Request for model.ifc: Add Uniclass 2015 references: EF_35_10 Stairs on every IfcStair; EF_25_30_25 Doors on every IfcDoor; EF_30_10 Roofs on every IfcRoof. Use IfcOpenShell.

First a look at what the model holds.

```python
import ifcopenshell

model = ifcopenshell.open("model.ifc")
print(model.schema)
print("classifications:", [c.Name for c in model.by_type("IfcClassification")])
for ifc_class in ("IfcDoor", "IfcRoof", "IfcStair", "IfcWall", "IfcWindow"):
    print(ifc_class, len(model.by_type(ifc_class)))
```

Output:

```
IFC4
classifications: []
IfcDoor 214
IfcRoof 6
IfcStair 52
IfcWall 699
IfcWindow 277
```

```python
import ifcopenshell
import ifcopenshell.api.classification

model = ifcopenshell.open("model.ifc")

system = ifcopenshell.api.classification.add_classification(model, classification="Uniclass 2015")

codes = {
    "IfcStair": ("EF_35_10", "Stairs"),
    "IfcDoor": ("EF_25_30_25", "Doors"),
    "IfcRoof": ("EF_30_10", "Roofs"),
}
for ifc_class, (code, name) in codes.items():
    products = model.by_type(ifc_class)
    ifcopenshell.api.classification.add_reference(
        model, products=products, classification=system, identification=code, name=name
    )
    print(code, len(products))

model.write("model_updated.ifc")
```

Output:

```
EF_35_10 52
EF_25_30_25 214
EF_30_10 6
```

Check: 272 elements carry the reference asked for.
